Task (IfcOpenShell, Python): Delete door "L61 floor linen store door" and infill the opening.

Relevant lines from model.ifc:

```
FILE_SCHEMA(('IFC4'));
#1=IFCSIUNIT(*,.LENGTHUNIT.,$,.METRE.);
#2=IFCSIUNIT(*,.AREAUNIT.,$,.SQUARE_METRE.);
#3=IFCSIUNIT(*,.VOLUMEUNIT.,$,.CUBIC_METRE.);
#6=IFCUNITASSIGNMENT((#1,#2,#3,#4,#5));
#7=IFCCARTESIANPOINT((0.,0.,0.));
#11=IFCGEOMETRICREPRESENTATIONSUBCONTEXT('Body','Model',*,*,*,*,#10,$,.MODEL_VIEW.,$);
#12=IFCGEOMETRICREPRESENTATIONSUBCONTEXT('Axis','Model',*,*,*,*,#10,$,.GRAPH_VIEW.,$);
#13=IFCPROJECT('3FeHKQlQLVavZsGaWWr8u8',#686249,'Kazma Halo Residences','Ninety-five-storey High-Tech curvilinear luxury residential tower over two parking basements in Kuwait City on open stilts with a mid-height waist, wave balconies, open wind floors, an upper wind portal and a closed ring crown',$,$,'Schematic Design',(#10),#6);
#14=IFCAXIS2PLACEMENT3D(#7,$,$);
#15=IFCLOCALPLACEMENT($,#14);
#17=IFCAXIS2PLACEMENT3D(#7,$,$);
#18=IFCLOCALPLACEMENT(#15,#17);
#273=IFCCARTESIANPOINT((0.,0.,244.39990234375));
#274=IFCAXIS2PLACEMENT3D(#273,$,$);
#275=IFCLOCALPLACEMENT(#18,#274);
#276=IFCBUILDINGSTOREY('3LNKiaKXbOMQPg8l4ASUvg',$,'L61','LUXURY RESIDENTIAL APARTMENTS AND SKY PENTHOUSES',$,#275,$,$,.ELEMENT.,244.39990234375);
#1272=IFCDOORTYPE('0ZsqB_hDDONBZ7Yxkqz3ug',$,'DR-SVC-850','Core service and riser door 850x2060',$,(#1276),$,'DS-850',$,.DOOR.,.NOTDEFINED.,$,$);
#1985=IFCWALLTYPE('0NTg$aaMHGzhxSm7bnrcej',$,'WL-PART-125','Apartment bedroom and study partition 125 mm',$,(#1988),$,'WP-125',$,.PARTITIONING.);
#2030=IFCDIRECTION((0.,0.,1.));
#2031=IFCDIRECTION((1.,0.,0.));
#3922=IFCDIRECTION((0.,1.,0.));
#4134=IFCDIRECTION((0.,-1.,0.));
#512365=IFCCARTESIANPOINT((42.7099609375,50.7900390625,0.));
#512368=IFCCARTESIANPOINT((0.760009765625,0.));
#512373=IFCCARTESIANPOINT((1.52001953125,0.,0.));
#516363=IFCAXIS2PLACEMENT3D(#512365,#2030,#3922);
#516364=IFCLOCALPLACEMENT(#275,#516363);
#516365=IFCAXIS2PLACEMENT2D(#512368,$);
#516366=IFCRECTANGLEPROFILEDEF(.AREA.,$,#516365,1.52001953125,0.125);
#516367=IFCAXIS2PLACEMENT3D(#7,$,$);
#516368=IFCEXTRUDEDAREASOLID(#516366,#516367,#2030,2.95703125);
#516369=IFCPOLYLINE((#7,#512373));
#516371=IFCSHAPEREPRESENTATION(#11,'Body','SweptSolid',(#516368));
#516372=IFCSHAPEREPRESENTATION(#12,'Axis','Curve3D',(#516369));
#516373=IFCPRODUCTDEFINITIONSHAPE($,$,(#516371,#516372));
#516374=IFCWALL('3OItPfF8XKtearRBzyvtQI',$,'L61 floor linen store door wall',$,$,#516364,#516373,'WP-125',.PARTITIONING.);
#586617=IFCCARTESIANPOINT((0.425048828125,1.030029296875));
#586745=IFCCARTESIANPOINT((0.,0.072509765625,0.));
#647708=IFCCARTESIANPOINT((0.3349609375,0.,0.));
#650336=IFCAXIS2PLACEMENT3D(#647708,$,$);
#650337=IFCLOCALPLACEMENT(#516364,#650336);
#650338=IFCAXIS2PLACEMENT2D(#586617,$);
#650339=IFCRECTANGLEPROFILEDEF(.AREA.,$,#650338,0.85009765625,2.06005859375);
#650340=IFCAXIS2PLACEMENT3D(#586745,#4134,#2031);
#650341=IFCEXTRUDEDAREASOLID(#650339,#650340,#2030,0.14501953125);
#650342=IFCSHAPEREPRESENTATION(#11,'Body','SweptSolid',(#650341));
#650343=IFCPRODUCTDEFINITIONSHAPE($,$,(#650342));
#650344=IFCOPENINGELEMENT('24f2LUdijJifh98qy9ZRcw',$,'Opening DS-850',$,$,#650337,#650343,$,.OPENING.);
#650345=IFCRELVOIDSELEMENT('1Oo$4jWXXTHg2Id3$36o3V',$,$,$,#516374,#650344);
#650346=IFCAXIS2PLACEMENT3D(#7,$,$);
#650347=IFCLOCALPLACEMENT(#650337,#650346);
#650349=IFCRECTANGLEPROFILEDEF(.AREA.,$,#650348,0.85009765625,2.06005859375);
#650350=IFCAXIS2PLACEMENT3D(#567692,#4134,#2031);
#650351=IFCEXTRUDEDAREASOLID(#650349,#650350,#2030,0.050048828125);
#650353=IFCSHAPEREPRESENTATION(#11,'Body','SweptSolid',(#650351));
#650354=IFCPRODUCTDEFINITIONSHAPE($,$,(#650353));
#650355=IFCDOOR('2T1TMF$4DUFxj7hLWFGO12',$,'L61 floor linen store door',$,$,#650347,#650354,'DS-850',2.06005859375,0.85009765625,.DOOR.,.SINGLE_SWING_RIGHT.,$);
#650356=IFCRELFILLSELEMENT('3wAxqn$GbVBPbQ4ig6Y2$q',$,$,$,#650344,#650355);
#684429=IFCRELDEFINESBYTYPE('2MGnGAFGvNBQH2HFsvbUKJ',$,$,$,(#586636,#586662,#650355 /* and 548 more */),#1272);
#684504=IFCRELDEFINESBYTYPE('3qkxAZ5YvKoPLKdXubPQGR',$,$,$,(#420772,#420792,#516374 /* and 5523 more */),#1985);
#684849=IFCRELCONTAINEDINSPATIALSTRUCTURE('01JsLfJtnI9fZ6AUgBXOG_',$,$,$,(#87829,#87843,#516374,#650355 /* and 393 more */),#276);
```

```python
import ifcopenshell
import ifcopenshell.api.feature
import ifcopenshell.api.root
import ifcopenshell.geom
import ifcopenshell.util.shape

model = ifcopenshell.open("model.ifc")
settings = ifcopenshell.geom.settings()


def volume(element):
    """Net volume in cubic metres, openings subtracted."""
    shape = ifcopenshell.geom.create_shape(settings, element)
    return ifcopenshell.util.shape.get_volume(shape.geometry)


door = model.by_id(650355)
opening = door.FillsVoids[0].RelatingOpeningElement
wall = opening.VoidsElements[0].RelatingBuildingElement
before = volume(wall)

ifcopenshell.api.root.remove_product(model, product=door)
ifcopenshell.api.feature.remove_feature(model, feature=opening)

after = volume(wall)

print(f"wall volume {before:.3f} -> {after:.3f} m3")

model.write("model-out.ifc")
```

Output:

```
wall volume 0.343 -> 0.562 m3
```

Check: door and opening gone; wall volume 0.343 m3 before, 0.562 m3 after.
